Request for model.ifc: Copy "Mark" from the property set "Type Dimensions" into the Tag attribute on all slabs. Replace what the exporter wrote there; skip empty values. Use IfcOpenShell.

First a look at what the model holds.

```python
import ifcopenshell
import ifcopenshell.util.element

model = ifcopenshell.open("model.ifc")
print(model.schema)
slabs = model.by_type("IfcSlab")
print(len(slabs), "slabs")
for e in slabs[:8]:
    source = ifcopenshell.util.element.get_pset(e, "Type Dimensions", "Mark")
    target = e.Tag
    print(e.id(), repr(source), repr(target), sep=" | ")
```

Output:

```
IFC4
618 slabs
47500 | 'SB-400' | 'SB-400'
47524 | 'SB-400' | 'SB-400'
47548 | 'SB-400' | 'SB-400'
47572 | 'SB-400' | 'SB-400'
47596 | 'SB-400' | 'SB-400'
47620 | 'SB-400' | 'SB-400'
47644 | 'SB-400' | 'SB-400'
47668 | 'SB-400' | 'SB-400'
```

```python
import ifcopenshell
import ifcopenshell.util.element

model = ifcopenshell.open("model.ifc")

count = 0
for e in model.by_type("IfcSlab"):
    value = ifcopenshell.util.element.get_pset(e, "Type Dimensions", "Mark")
    current = e.Tag
    if not value or not value.strip() or current == value:
        continue
    e.Tag = value
    count += 1

print(count, "slabs updated")

model.write("model_rev.ifc")
```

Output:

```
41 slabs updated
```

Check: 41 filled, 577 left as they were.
